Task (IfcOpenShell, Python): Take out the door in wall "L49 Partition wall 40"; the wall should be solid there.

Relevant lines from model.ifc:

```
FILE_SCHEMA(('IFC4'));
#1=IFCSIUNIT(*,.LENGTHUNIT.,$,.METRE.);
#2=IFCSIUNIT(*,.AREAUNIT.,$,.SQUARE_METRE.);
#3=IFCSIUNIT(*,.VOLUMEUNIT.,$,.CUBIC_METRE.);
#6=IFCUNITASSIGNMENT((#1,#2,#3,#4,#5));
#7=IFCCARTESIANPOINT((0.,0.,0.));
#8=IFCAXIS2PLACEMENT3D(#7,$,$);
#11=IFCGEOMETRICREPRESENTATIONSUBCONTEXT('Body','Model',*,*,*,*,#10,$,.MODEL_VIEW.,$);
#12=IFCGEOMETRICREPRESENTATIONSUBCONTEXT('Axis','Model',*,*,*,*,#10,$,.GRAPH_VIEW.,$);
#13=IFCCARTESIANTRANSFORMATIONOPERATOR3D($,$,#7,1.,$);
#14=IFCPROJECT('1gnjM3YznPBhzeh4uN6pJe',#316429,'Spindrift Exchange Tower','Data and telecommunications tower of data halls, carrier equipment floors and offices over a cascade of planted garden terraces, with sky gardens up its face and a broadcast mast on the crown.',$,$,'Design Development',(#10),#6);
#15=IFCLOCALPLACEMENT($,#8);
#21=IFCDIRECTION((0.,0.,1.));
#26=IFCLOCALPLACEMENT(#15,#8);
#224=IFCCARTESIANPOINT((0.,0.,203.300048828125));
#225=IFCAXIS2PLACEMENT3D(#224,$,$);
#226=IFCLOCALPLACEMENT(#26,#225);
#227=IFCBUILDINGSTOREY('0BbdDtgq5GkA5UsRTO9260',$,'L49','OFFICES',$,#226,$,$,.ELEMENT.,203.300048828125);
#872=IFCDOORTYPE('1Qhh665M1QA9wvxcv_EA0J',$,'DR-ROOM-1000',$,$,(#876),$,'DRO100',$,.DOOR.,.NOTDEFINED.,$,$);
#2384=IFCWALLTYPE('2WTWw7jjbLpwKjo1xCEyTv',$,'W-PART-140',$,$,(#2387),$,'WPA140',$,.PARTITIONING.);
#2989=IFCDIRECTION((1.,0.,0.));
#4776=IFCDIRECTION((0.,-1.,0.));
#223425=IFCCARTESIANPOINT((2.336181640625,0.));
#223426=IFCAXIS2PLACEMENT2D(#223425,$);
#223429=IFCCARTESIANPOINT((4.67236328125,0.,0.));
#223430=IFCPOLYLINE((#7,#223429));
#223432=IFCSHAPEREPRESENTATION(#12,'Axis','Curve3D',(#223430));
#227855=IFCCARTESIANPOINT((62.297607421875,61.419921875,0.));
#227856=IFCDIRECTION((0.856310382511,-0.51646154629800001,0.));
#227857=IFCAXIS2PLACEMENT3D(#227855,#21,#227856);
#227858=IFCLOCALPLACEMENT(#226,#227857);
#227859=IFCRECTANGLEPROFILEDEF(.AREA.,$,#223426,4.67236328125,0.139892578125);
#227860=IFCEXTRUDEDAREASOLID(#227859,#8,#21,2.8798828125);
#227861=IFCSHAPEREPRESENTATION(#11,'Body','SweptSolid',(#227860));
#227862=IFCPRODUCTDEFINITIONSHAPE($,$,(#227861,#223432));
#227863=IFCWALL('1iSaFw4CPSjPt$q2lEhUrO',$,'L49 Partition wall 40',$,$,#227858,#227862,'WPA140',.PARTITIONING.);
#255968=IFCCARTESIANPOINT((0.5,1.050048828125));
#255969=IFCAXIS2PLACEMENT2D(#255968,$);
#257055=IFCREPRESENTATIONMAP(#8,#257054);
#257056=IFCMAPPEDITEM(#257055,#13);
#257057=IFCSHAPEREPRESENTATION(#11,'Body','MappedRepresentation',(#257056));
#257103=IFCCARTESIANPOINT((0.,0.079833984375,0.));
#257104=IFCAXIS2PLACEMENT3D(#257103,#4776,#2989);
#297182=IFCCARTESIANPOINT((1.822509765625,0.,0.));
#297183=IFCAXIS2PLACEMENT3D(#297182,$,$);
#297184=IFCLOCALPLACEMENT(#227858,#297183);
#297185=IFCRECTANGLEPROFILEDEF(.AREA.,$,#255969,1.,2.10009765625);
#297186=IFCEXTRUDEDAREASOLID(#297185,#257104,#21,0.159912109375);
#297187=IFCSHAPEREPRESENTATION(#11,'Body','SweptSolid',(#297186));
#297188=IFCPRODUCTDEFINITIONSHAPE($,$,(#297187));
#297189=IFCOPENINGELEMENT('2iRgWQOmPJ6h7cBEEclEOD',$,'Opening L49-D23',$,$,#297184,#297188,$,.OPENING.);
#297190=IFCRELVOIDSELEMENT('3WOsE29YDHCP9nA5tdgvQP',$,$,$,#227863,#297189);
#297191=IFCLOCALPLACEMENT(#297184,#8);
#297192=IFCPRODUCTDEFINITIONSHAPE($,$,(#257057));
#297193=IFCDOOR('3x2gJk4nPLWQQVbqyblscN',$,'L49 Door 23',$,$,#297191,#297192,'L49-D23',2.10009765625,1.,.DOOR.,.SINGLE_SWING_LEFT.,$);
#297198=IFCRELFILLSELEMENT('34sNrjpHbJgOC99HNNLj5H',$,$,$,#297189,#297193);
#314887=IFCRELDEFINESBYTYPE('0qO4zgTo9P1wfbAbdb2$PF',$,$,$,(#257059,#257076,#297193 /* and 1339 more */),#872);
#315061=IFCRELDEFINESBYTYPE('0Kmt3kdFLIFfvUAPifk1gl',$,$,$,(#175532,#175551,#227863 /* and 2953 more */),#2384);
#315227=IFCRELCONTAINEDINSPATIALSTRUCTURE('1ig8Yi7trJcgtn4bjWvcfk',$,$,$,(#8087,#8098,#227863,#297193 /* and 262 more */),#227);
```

```python
import ifcopenshell
import ifcopenshell.api.feature
import ifcopenshell.api.root
import ifcopenshell.geom
import ifcopenshell.util.shape

model = ifcopenshell.open("model.ifc")
settings = ifcopenshell.geom.settings()


def volume(element):
    """Net volume in cubic metres, openings subtracted."""
    shape = ifcopenshell.geom.create_shape(settings, element)
    return ifcopenshell.util.shape.get_volume(shape.geometry)


door = model.by_id(297193)
opening = door.FillsVoids[0].RelatingOpeningElement
wall = opening.VoidsElements[0].RelatingBuildingElement
before = volume(wall)

ifcopenshell.api.root.remove_product(model, product=door)
ifcopenshell.api.feature.remove_feature(model, feature=opening)

after = volume(wall)

print(f"wall volume {before:.3f} -> {after:.3f} m3")

model.write("model_rev.ifc")
```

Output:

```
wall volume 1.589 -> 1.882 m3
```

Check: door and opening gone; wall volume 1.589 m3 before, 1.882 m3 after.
